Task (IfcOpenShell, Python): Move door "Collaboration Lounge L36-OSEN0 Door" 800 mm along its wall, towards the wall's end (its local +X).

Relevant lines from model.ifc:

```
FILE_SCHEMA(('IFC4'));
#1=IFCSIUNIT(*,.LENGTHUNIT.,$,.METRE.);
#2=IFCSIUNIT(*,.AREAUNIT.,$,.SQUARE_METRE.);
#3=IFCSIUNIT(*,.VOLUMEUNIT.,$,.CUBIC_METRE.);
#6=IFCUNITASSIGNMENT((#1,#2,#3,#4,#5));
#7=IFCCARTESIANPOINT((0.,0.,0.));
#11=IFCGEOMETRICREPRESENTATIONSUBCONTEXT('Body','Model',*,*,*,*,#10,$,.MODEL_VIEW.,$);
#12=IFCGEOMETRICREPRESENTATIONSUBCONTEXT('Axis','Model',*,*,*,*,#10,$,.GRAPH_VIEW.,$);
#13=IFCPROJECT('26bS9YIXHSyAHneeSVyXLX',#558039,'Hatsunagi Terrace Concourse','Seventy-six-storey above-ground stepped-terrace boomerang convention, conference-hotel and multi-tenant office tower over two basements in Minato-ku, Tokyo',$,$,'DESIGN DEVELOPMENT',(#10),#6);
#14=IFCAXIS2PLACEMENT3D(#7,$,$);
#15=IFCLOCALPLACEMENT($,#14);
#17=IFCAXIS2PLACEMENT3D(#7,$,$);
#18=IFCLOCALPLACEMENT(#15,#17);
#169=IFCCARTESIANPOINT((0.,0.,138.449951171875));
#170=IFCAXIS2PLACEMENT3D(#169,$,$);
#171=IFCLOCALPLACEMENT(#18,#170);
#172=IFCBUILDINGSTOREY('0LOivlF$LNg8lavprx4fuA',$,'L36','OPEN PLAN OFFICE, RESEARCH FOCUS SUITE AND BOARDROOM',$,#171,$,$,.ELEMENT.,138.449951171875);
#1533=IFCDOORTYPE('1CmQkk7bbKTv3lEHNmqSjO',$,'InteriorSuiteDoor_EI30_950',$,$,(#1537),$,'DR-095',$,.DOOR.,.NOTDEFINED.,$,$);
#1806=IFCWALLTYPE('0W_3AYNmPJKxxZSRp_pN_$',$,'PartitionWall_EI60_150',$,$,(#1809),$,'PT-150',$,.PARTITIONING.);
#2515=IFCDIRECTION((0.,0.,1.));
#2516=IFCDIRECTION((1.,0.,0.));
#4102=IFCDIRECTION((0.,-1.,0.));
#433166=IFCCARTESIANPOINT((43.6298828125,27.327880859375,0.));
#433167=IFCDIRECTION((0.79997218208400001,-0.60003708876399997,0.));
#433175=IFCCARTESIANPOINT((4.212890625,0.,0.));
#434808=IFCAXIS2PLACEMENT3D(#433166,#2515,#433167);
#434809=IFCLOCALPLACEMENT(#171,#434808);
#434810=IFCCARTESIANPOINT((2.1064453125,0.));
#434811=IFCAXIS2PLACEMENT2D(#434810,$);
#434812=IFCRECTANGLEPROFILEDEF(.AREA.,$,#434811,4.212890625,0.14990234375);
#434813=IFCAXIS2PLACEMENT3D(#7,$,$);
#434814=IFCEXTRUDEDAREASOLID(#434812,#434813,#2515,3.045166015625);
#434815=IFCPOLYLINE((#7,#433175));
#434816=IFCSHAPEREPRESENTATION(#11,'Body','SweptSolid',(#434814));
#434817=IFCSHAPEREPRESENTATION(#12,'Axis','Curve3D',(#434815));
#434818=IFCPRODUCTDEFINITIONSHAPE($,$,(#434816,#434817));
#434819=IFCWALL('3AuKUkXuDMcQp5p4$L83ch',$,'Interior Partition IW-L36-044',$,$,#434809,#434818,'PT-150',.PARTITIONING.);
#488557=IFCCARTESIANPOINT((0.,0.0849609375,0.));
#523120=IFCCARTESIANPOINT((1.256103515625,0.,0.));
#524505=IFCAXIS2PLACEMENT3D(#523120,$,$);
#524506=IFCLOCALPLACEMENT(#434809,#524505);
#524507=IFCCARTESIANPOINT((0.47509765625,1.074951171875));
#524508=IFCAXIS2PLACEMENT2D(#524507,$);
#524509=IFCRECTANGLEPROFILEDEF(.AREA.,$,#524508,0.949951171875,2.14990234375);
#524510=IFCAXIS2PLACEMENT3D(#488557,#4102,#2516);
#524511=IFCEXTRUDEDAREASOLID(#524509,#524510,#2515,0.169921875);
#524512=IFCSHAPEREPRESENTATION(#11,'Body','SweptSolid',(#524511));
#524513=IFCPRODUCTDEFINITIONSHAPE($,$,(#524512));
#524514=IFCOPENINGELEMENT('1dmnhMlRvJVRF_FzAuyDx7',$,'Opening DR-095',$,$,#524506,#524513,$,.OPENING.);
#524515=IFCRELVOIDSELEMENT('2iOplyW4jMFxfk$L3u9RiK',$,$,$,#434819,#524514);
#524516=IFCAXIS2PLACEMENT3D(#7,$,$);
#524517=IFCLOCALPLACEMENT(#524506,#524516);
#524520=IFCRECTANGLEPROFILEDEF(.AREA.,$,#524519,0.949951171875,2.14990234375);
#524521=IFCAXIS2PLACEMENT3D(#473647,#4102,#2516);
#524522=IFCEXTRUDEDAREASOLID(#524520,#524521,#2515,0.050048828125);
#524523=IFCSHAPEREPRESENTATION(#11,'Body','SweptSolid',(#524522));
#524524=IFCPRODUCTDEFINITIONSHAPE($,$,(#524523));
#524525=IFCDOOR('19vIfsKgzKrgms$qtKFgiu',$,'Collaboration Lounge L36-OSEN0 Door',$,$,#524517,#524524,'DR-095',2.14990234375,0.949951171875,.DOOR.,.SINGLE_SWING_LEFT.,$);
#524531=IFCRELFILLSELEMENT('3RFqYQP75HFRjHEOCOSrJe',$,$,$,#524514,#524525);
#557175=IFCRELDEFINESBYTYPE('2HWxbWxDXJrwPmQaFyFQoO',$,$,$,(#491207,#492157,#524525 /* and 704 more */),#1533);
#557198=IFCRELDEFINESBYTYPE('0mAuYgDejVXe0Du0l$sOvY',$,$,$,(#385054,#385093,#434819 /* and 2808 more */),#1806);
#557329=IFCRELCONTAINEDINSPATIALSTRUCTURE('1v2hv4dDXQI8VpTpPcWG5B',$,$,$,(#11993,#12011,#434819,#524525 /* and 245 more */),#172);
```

```python
import ifcopenshell
import ifcopenshell.api.geometry
import ifcopenshell.util.placement
import ifcopenshell.util.unit

model = ifcopenshell.open("model.ifc")
unit_scale = ifcopenshell.util.unit.calculate_unit_scale(model)

door = model.by_guid("19vIfsKgzKrgms$qtKFgiu")
opening = door.FillsVoids[0].RelatingOpeningElement
wall = opening.VoidsElements[0].RelatingBuildingElement

wall_matrix = ifcopenshell.util.placement.get_local_placement(wall.ObjectPlacement)
shift = wall_matrix[:3, 0] * 0.8 / unit_scale
before = ifcopenshell.util.placement.get_local_placement(door.ObjectPlacement)[:3, 3].copy()

# The door is placed relative to its opening, so it follows when the opening moves.
matrix = ifcopenshell.util.placement.get_local_placement(opening.ObjectPlacement)
matrix[:3, 3] += shift
ifcopenshell.api.geometry.edit_object_placement(
    model, product=opening, matrix=matrix, is_si=False, should_transform_children=True
)

after = ifcopenshell.util.placement.get_local_placement(door.ObjectPlacement)[:3, 3]
print("door moved by", (after - before).round(3) + 0.0)

model.write("model_updated.ifc")
```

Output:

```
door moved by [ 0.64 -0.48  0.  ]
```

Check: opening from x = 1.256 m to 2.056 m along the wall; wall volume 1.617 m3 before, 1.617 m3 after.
